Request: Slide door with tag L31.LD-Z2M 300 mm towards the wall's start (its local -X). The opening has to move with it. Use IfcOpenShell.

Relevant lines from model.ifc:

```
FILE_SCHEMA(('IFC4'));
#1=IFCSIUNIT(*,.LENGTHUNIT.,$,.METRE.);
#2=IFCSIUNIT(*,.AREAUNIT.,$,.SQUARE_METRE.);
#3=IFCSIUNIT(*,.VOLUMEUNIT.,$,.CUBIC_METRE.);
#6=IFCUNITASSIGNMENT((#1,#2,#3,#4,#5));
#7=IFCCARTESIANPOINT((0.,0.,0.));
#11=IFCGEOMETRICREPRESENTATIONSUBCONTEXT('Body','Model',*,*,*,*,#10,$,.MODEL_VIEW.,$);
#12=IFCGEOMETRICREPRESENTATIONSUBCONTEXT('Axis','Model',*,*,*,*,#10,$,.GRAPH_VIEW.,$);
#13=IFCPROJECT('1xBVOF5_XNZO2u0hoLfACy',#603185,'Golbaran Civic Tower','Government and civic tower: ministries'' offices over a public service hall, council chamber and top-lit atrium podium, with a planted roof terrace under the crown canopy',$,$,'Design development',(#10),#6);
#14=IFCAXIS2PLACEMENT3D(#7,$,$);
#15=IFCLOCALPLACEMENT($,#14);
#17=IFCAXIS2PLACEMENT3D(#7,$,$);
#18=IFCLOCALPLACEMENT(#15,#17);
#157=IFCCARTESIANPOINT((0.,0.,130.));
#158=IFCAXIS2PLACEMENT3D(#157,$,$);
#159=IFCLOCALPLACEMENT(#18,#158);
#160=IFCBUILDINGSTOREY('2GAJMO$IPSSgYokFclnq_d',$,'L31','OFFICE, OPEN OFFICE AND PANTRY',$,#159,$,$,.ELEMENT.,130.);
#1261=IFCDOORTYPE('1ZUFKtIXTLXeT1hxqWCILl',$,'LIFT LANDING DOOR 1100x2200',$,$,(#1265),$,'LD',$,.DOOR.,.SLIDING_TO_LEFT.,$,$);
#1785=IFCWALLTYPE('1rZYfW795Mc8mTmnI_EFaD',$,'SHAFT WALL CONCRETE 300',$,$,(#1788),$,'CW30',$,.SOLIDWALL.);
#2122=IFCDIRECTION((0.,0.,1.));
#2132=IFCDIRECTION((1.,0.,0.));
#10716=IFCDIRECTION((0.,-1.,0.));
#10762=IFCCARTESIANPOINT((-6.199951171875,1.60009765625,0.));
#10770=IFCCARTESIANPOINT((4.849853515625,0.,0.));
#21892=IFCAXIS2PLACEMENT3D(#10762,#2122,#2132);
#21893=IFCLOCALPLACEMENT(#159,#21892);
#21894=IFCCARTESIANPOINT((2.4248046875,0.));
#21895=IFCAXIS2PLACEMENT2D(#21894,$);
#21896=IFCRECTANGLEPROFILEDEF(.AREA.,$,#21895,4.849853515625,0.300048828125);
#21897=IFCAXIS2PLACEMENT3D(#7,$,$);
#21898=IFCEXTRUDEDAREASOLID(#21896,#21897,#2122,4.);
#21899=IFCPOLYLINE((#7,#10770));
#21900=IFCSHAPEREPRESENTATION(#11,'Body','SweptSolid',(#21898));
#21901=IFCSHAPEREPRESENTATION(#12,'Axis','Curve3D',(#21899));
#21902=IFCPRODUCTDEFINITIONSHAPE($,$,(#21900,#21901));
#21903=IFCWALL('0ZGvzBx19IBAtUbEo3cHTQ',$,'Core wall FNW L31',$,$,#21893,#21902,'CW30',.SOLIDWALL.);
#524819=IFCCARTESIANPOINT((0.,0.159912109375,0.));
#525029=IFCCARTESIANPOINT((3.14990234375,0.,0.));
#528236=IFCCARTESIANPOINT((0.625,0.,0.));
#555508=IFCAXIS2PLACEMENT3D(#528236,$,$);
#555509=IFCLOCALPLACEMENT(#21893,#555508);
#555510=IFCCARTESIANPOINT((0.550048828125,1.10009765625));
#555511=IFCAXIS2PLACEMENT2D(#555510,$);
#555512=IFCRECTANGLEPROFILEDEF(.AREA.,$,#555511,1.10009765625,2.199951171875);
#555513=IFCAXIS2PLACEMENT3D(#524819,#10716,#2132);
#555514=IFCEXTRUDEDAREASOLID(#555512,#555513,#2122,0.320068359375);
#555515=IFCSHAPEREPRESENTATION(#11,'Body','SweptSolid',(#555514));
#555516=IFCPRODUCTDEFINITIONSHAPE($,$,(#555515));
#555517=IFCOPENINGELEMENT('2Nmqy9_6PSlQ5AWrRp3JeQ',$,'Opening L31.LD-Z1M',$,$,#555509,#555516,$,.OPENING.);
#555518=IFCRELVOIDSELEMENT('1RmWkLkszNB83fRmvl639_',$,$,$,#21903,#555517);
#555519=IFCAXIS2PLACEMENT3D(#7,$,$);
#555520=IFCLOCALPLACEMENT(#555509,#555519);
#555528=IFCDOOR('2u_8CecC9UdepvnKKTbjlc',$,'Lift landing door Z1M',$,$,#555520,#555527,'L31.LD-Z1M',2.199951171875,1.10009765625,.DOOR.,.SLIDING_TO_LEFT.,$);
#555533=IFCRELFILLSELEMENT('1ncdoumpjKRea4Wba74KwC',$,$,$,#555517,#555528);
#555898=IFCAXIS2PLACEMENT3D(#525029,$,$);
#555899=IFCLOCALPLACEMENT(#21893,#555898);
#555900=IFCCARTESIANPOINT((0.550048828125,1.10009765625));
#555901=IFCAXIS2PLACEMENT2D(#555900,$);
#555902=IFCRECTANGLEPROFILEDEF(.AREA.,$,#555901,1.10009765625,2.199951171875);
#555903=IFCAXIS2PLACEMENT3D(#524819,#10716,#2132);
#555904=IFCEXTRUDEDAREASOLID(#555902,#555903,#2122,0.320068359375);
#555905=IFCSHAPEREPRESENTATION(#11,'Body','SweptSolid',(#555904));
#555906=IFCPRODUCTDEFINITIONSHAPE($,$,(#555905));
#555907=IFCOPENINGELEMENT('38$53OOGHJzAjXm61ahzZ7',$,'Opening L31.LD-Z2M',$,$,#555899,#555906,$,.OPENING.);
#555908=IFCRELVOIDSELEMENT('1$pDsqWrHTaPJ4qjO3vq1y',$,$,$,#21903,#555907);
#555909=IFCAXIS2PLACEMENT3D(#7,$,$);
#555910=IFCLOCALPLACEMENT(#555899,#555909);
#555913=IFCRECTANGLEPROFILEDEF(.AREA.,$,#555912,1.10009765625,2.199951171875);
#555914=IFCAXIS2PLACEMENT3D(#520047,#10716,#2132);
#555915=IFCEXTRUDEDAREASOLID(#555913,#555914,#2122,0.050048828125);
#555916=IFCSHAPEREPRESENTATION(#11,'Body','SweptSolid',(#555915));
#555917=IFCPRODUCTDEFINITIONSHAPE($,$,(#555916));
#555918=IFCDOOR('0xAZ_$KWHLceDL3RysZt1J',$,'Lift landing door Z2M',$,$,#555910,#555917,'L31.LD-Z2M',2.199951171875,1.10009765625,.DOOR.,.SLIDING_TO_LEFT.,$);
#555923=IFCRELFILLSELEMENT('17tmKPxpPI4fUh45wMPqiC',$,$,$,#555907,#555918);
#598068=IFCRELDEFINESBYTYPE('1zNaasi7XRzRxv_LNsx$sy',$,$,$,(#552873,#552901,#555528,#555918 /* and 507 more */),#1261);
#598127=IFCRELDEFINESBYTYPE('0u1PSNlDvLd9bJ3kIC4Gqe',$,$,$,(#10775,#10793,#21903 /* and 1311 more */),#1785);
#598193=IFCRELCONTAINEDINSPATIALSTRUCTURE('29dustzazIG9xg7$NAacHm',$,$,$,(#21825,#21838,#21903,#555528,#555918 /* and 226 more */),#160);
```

```python
import ifcopenshell
import ifcopenshell.api.geometry
import ifcopenshell.util.placement
import ifcopenshell.util.unit

model = ifcopenshell.open("model.ifc")
unit_scale = ifcopenshell.util.unit.calculate_unit_scale(model)

door = model.by_guid("0xAZ_$KWHLceDL3RysZt1J")
opening = door.FillsVoids[0].RelatingOpeningElement
wall = opening.VoidsElements[0].RelatingBuildingElement

wall_matrix = ifcopenshell.util.placement.get_local_placement(wall.ObjectPlacement)
shift = wall_matrix[:3, 0] * -0.3 / unit_scale
before = ifcopenshell.util.placement.get_local_placement(door.ObjectPlacement)[:3, 3].copy()

# The door is placed relative to its opening, so it follows when the opening moves.
matrix = ifcopenshell.util.placement.get_local_placement(opening.ObjectPlacement)
matrix[:3, 3] += shift
ifcopenshell.api.geometry.edit_object_placement(
    model, product=opening, matrix=matrix, is_si=False, should_transform_children=True
)

after = ifcopenshell.util.placement.get_local_placement(door.ObjectPlacement)[:3, 3]
print("door moved by", (after - before).round(3) + 0.0)

model.write("model_updated.ifc")
```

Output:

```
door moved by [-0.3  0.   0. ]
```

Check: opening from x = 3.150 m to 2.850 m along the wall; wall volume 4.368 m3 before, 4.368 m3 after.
